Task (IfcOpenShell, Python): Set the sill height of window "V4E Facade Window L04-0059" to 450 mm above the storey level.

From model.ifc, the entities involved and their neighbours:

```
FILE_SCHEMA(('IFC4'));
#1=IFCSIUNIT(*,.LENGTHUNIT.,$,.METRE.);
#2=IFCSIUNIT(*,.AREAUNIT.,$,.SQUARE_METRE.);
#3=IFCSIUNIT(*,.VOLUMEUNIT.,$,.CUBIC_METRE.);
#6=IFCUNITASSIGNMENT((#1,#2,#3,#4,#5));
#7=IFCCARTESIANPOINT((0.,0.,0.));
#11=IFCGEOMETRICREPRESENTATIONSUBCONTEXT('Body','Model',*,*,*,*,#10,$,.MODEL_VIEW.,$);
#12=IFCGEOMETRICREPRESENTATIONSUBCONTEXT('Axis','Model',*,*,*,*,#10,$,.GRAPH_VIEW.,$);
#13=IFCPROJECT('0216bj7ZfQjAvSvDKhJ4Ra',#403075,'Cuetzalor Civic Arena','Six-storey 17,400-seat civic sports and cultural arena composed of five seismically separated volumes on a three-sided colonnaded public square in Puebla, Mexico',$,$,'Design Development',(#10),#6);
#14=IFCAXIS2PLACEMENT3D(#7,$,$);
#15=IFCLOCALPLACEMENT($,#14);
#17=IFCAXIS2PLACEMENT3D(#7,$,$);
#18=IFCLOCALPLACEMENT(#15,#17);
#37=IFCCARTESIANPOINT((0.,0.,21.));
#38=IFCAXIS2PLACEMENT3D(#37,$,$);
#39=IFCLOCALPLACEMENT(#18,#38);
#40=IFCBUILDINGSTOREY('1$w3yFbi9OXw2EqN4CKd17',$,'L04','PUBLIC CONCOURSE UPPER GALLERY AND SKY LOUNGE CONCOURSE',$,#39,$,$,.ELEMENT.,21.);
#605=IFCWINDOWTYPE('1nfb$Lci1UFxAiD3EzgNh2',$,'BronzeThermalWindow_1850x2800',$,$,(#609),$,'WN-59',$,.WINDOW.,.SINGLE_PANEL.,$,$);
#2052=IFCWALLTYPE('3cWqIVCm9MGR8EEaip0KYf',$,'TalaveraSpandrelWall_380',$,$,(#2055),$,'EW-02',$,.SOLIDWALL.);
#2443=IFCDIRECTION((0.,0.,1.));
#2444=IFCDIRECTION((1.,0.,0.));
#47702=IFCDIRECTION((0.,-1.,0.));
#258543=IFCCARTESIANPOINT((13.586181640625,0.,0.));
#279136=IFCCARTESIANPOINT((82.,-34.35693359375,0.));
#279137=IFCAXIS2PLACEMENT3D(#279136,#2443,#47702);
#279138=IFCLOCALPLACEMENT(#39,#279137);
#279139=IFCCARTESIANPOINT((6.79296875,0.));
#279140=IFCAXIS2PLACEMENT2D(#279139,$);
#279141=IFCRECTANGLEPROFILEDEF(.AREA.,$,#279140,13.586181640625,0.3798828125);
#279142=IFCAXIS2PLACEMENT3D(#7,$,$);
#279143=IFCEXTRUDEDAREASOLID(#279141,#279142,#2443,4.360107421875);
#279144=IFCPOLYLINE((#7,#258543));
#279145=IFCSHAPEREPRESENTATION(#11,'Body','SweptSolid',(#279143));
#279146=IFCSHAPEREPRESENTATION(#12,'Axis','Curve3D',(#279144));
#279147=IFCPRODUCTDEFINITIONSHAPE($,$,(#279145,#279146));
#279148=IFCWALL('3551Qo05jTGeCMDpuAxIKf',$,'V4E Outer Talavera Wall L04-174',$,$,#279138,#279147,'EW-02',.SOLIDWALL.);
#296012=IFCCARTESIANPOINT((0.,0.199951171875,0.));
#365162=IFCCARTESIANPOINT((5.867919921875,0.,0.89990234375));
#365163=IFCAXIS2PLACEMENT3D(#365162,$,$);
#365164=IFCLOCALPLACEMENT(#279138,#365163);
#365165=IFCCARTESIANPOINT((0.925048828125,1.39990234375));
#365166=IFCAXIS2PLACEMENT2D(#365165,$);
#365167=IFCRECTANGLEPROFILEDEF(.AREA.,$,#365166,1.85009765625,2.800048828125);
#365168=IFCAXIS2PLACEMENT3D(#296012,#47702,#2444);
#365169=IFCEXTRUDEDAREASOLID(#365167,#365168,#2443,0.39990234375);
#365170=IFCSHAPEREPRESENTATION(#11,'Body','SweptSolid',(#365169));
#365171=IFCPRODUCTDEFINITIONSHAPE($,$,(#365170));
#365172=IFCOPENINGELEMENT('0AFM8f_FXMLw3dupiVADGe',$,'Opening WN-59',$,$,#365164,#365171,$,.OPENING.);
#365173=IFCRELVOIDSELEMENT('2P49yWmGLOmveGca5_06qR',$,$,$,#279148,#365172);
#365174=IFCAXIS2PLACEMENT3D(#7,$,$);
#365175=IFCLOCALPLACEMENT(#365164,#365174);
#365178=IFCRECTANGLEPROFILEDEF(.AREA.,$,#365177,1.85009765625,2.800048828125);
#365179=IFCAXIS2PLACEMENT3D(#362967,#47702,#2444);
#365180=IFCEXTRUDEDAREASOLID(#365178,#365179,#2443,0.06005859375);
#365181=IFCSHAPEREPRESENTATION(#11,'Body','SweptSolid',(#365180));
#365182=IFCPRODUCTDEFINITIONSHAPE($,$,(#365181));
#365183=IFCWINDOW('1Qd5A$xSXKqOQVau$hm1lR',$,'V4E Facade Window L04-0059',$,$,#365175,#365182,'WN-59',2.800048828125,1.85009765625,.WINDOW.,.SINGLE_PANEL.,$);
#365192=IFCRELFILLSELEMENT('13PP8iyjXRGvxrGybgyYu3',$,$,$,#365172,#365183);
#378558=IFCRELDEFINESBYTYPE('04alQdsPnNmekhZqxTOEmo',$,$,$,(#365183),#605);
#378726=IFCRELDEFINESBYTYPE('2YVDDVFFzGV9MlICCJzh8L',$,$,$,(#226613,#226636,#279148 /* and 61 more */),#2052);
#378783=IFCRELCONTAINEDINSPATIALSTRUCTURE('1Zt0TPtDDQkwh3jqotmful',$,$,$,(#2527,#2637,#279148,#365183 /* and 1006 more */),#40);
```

```python
import numpy as np
import ifcopenshell
import ifcopenshell.api.geometry
import ifcopenshell.geom
import ifcopenshell.util.element
import ifcopenshell.util.placement
import ifcopenshell.util.shape
import ifcopenshell.util.unit

model = ifcopenshell.open("model.ifc")
unit_scale = ifcopenshell.util.unit.calculate_unit_scale(model)

window = model.by_guid("1Qd5A$xSXKqOQVau$hm1lR")
opening = window.FillsVoids[0].RelatingOpeningElement
storey = ifcopenshell.util.element.get_container(window, ifc_class="IfcBuildingStorey")
level = ifcopenshell.util.placement.get_local_placement(storey.ObjectPlacement)[2, 3]

# The opening's origin need not be at the sill, so measure its lowest point.
shape = ifcopenshell.geom.create_shape(ifcopenshell.geom.settings(), opening)
bottom = ifcopenshell.util.shape.get_shape_bottom_elevation(shape, shape.geometry) / unit_scale
dz = level + 0.45 - bottom

shift = np.array([0.0, 0.0, dz])
# The window is placed relative to its opening, so it follows when the opening moves.
matrix = ifcopenshell.util.placement.get_local_placement(opening.ObjectPlacement)
matrix[:3, 3] += shift
ifcopenshell.api.geometry.edit_object_placement(
    model, product=opening, matrix=matrix, is_si=False, should_transform_children=True
)

print(f"moved by {dz * unit_scale:+.3f} m")

model.write("model_edited.ifc")
```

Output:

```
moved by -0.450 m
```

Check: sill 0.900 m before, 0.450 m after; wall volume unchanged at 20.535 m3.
